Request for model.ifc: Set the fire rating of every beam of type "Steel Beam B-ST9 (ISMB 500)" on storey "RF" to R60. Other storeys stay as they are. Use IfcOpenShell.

First a look at what the model holds.

```python
import ifcopenshell
import ifcopenshell.util.element

model = ifcopenshell.open("model.ifc")
print(model.schema)
storey = next(s for s in model.by_type("IfcBuildingStorey") if s.Name == "RF")
beams = [e for e in ifcopenshell.util.element.get_decomposition(storey) if e.is_a("IfcBeam")]
seen = {}
for e in beams:
    element_type = ifcopenshell.util.element.get_type(e)
    key = (element_type.Name if element_type != e and element_type else None, ifcopenshell.util.element.get_pset(e, "Pset_BeamCommon", "FireRating"))
    seen[key] = seen.get(key, 0) + 1
for (name, value), count in sorted(seen.items(), key=str):
    print(count, "x", name, "|", value)
```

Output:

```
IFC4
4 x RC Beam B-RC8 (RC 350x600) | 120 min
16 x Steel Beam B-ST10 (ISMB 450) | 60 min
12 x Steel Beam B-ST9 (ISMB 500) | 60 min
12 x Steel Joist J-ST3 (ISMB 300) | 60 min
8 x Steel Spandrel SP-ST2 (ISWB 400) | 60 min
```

```python
import ifcopenshell
import ifcopenshell.api.pset
import ifcopenshell.util.element

model = ifcopenshell.open("model.ifc")

storey = next(s for s in model.by_type("IfcBuildingStorey") if s.Name == "RF")
beams = [e for e in ifcopenshell.util.element.get_decomposition(storey) if e.is_a("IfcBeam")]

count = 0
for e in beams:
    element_type = ifcopenshell.util.element.get_type(e)
    if element_type in (None, e) or element_type.Name != "Steel Beam B-ST9 (ISMB 500)":
        continue
    # add_pset returns the element's existing set when there is one.
    pset = ifcopenshell.api.pset.add_pset(model, product=e, name="Pset_BeamCommon")
    ifcopenshell.api.pset.edit_pset(model, pset=pset, properties={"FireRating": "R60"})
    count += 1

print(count, "beams updated")

model.write("model_edited.ifc")
```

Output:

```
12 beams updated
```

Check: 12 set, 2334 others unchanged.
